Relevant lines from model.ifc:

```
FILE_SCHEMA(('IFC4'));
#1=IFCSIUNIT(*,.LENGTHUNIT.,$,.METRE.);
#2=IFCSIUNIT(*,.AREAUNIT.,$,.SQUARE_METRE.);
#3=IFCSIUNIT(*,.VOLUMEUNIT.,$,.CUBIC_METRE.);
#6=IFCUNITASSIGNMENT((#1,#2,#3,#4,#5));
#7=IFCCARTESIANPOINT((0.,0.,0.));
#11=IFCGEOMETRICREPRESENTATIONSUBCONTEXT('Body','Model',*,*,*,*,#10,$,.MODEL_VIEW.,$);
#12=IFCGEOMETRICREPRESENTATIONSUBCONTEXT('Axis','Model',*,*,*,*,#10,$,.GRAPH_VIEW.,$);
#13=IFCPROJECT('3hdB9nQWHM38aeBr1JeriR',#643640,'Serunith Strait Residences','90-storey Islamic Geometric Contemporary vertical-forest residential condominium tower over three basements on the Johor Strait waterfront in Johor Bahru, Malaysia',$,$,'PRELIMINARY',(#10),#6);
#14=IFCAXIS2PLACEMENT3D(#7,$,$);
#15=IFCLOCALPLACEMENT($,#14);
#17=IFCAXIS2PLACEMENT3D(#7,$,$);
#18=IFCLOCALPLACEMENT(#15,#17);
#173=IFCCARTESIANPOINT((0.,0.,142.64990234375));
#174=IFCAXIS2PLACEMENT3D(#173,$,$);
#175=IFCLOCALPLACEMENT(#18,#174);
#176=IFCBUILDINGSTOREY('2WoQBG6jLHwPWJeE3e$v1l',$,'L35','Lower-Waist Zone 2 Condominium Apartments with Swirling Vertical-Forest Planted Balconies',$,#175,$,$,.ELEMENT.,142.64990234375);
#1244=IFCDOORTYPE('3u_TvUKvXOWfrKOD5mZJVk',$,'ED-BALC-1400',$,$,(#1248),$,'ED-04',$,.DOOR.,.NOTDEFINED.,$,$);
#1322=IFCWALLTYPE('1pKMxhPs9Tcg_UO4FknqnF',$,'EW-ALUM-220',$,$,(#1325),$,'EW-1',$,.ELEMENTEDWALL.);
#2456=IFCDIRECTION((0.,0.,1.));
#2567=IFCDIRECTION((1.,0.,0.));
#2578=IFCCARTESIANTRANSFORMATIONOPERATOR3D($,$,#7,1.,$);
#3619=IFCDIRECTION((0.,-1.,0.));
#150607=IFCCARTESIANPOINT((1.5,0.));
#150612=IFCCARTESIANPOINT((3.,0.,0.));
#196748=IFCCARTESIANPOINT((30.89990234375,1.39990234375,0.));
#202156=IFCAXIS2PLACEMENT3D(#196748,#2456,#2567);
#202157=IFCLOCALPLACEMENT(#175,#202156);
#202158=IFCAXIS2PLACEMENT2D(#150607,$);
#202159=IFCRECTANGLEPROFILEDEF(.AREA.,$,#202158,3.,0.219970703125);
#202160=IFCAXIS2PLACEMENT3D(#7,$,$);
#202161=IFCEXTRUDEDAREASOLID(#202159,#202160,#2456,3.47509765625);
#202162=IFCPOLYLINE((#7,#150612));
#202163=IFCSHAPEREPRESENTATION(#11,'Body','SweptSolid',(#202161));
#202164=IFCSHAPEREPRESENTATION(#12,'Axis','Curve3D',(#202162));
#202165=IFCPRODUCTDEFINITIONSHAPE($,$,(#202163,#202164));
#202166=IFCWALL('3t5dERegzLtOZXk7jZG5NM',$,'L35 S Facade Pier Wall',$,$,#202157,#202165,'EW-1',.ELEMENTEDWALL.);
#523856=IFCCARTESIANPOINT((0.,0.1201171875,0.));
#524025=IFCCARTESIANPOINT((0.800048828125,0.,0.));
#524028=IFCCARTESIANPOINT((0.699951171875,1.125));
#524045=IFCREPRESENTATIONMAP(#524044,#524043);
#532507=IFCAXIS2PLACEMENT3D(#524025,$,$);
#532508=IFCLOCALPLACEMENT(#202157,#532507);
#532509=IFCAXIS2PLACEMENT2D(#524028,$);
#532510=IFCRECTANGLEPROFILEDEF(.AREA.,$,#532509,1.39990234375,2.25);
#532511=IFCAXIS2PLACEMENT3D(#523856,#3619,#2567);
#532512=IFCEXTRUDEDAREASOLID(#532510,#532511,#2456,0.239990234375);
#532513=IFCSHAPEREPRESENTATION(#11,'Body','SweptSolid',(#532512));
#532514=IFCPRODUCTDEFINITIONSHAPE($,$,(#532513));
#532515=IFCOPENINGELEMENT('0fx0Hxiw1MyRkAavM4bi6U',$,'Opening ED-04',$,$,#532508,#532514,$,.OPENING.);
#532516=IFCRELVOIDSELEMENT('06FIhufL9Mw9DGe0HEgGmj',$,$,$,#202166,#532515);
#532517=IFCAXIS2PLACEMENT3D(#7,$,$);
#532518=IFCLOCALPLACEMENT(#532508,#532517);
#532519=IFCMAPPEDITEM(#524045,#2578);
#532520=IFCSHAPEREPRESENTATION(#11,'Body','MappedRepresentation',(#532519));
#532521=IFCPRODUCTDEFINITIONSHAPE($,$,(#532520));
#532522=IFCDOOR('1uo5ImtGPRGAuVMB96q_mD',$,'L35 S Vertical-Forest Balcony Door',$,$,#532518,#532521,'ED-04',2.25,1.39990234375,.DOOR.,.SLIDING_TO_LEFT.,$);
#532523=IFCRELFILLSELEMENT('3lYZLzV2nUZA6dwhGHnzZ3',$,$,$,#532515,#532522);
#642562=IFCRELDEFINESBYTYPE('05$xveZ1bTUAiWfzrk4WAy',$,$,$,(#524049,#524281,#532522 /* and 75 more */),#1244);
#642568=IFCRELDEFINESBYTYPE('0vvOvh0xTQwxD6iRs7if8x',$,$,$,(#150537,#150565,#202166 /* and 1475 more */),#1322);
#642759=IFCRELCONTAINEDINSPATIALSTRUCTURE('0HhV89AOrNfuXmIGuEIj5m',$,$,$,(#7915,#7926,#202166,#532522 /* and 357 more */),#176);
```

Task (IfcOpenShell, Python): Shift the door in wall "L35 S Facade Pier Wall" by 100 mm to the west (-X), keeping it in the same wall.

```python
import ifcopenshell
import ifcopenshell.api.geometry
import ifcopenshell.util.placement
import ifcopenshell.util.unit

model = ifcopenshell.open("model.ifc")
unit_scale = ifcopenshell.util.unit.calculate_unit_scale(model)

door = model.by_guid("1uo5ImtGPRGAuVMB96q_mD")
opening = door.FillsVoids[0].RelatingOpeningElement
wall = opening.VoidsElements[0].RelatingBuildingElement

wall_matrix = ifcopenshell.util.placement.get_local_placement(wall.ObjectPlacement)
shift = wall_matrix[:3, 0] * -0.1 / unit_scale
before = ifcopenshell.util.placement.get_local_placement(door.ObjectPlacement)[:3, 3].copy()

# The door is placed relative to its opening, so it follows when the opening moves.
matrix = ifcopenshell.util.placement.get_local_placement(opening.ObjectPlacement)
matrix[:3, 3] += shift
ifcopenshell.api.geometry.edit_object_placement(
    model, product=opening, matrix=matrix, is_si=False, should_transform_children=True
)

after = ifcopenshell.util.placement.get_local_placement(door.ObjectPlacement)[:3, 3]
print("door moved by", (after - before).round(3) + 0.0)

model.write("model_v2.ifc")
```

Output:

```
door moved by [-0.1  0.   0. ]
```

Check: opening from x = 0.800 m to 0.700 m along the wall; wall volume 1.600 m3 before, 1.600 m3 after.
